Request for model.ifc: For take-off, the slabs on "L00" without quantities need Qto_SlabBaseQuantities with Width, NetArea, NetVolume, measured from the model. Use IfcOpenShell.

First a look at what the model holds.

```python
import ifcopenshell
import ifcopenshell.util.element
import ifcopenshell.util.unit

model = ifcopenshell.open("model.ifc")
print(model.schema)
for unit_type in ("LENGTHUNIT", "AREAUNIT", "VOLUMEUNIT"):
    print(unit_type, ifcopenshell.util.unit.calculate_unit_scale(model, unit_type))
storey = next(s for s in model.by_type("IfcBuildingStorey") if s.Name == "L00")
slabs = [e for e in ifcopenshell.util.element.get_decomposition(storey) if e.is_a("IfcSlab")]
for e in sorted(slabs, key=lambda e: e.id()):
    print(e.id(), e.is_a(), e.Name, list(ifcopenshell.util.element.get_psets(e, qtos_only=True)), sep=" | ")
```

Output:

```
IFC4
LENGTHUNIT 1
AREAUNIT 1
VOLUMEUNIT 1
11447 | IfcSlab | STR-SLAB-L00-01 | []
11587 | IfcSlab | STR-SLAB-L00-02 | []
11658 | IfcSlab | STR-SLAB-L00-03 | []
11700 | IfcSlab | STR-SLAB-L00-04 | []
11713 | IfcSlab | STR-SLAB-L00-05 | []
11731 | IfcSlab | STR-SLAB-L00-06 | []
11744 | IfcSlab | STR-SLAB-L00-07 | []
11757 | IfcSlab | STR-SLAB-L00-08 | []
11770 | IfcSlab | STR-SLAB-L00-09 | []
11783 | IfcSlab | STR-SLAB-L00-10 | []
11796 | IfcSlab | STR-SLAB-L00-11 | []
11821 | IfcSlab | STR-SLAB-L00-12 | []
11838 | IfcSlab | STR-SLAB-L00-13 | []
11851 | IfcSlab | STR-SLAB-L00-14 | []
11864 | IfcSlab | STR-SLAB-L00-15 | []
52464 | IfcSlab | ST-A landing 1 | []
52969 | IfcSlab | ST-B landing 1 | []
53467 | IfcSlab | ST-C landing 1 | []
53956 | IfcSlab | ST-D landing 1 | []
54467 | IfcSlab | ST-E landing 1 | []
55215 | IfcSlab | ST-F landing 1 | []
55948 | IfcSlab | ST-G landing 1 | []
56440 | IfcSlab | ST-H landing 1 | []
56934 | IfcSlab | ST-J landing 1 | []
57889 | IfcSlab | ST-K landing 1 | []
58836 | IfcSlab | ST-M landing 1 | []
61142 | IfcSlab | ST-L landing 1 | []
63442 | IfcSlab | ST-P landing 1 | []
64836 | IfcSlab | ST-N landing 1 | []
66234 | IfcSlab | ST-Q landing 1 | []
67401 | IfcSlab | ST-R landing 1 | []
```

```python
import ifcopenshell
import ifcopenshell.api.pset
import ifcopenshell.geom
import ifcopenshell.util.element
import ifcopenshell.util.shape
import ifcopenshell.util.unit

model = ifcopenshell.open("model.ifc")
unit_scale = ifcopenshell.util.unit.calculate_unit_scale(model)
area_scale = ifcopenshell.util.unit.calculate_unit_scale(model, "AREAUNIT")
volume_scale = ifcopenshell.util.unit.calculate_unit_scale(model, "VOLUMEUNIT")
settings = ifcopenshell.geom.settings()

storey = next(s for s in model.by_type("IfcBuildingStorey") if s.Name == "L00")
slabs = [e for e in ifcopenshell.util.element.get_decomposition(storey) if e.is_a("IfcSlab")]

for e in sorted(slabs, key=lambda e: e.id()):
    if ifcopenshell.util.element.get_psets(e, qtos_only=True, should_inherit=False):
        continue
    # Geometry comes back in metres, in the element's own axes.
    shape = ifcopenshell.geom.create_shape(settings, e)
    values = {
        "Width": ifcopenshell.util.shape.get_z(shape.geometry) / unit_scale,
        "NetArea": ifcopenshell.util.shape.get_footprint_area(shape.geometry) / area_scale,
        "NetVolume": ifcopenshell.util.shape.get_volume(shape.geometry) / volume_scale,
    }
    qto = ifcopenshell.api.pset.add_qto(model, product=e, name="Qto_SlabBaseQuantities")
    ifcopenshell.api.pset.edit_qto(model, qto=qto, properties=values)
    print(e.id(), {k: round(v, 3) for k, v in values.items()})

model.write("model_rev.ifc")
```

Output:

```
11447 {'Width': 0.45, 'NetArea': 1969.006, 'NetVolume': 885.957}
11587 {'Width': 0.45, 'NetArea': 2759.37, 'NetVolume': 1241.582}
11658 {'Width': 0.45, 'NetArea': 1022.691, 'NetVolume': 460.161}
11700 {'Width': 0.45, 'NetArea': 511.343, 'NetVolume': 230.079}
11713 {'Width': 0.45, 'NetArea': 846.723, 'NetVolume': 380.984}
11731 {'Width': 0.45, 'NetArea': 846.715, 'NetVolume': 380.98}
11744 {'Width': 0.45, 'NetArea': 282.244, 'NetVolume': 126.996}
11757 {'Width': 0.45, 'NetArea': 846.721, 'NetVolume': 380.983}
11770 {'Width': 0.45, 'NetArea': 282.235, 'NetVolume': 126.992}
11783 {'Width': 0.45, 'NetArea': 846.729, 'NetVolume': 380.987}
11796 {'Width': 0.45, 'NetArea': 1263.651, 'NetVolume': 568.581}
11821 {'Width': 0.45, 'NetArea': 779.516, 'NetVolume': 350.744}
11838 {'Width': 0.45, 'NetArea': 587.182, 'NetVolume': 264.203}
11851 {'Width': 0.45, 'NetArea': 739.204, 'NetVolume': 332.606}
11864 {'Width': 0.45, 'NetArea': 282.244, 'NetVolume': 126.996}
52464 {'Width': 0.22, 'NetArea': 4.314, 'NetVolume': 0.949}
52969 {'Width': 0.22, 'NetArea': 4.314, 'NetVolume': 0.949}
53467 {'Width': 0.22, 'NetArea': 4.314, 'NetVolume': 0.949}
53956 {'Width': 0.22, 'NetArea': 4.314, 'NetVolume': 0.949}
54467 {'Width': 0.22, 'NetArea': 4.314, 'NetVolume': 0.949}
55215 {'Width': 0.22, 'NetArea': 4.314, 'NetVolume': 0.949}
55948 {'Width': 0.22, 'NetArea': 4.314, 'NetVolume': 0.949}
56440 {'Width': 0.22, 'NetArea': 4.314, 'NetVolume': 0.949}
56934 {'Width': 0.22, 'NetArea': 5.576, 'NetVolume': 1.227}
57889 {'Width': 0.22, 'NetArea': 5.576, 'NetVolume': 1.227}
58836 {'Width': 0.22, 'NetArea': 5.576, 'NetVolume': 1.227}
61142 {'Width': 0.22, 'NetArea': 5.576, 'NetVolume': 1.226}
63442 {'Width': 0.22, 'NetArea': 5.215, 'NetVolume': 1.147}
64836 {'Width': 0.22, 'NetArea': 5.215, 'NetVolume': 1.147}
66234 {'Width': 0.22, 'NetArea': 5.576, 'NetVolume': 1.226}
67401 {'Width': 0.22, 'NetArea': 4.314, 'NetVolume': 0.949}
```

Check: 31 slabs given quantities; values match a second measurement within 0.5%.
